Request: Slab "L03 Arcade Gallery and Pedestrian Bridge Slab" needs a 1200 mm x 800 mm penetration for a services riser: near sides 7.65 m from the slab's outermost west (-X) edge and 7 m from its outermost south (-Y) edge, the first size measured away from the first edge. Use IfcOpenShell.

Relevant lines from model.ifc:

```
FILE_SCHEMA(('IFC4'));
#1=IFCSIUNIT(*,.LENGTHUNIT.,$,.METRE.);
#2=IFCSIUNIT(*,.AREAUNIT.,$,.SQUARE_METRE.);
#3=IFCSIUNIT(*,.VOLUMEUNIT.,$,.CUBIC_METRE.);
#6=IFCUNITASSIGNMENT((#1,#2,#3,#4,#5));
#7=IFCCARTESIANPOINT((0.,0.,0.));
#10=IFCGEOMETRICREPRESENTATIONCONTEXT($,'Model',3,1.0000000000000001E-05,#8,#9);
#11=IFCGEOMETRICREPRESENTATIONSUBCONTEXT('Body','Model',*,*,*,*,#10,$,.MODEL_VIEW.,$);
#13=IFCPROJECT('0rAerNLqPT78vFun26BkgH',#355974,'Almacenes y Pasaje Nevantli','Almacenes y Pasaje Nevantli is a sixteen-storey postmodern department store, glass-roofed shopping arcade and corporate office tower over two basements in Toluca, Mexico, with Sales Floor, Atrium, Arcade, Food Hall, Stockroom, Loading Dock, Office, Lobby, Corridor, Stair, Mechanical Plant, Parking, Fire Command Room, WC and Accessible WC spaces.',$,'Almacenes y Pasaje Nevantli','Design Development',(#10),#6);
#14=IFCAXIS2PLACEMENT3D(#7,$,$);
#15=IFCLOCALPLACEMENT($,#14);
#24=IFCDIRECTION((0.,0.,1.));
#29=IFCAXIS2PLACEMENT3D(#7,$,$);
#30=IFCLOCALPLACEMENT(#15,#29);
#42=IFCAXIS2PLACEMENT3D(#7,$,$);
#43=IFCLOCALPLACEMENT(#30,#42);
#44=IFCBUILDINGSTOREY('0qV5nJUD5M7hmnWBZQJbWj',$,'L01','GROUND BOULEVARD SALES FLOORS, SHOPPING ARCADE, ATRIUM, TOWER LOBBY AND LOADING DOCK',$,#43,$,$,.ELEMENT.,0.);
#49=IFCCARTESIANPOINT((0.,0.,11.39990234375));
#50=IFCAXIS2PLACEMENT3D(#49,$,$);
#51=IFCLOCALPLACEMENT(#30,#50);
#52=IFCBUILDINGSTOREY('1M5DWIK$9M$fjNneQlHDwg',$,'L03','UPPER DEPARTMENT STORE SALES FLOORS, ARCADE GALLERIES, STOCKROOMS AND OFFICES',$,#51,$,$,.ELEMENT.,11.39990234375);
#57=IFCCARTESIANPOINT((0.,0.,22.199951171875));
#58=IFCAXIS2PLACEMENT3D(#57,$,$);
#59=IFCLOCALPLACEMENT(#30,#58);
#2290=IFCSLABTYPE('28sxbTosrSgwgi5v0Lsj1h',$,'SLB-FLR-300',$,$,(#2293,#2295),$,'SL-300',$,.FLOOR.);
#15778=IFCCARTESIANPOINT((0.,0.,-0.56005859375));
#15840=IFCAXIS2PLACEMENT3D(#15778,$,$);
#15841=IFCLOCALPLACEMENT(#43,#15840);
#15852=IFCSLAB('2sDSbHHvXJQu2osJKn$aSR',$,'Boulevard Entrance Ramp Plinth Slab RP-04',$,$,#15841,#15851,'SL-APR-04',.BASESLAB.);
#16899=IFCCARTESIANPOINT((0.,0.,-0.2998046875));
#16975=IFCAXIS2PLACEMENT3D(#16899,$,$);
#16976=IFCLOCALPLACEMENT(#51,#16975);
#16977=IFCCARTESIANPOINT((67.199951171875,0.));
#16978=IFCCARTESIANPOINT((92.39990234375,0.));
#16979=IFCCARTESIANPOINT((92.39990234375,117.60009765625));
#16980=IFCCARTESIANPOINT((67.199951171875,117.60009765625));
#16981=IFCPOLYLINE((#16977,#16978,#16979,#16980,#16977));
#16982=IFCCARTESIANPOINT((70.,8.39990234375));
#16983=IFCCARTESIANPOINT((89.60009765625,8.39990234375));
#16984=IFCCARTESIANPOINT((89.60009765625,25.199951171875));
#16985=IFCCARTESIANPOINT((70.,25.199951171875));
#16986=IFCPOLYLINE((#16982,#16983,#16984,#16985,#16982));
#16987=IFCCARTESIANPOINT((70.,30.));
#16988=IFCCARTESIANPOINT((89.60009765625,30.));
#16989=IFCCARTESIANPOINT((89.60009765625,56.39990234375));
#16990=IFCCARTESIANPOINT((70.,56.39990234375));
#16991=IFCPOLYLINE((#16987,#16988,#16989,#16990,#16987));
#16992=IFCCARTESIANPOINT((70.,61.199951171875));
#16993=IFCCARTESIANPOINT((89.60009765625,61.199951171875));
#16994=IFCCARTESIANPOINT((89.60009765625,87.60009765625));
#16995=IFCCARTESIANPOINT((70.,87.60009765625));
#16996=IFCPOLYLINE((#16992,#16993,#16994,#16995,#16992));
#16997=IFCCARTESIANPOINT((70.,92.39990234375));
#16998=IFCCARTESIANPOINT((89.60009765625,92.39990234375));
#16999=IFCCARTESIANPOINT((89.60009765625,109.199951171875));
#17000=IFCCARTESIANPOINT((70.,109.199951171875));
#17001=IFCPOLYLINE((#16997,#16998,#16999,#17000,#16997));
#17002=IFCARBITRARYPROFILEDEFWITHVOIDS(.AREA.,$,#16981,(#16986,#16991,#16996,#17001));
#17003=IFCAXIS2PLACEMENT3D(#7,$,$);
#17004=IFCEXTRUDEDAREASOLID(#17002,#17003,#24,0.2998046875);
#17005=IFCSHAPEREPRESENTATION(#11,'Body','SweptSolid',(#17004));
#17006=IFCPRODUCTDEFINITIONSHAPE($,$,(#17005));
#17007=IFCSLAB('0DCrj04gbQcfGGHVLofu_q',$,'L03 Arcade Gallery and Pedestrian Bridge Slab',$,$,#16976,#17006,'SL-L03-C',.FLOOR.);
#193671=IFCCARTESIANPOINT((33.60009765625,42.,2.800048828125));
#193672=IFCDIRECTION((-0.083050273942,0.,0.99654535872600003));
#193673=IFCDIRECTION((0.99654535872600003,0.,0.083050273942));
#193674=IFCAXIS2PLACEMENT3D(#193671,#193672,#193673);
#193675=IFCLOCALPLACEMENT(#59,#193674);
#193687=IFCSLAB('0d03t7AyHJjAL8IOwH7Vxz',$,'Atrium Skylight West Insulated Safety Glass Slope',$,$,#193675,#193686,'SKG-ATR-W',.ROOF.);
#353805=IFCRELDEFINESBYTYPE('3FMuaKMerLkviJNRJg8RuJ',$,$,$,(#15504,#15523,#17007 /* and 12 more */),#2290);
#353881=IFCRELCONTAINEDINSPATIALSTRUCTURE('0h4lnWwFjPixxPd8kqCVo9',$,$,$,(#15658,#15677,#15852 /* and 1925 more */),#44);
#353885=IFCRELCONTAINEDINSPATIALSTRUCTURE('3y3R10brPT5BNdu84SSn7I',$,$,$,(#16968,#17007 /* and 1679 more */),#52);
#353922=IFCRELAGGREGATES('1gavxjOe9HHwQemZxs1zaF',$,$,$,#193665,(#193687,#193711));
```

```python
import numpy as np
import ifcopenshell
import ifcopenshell.api.feature
import ifcopenshell.api.geometry
import ifcopenshell.api.root
import ifcopenshell.geom
import ifcopenshell.util.placement
import ifcopenshell.util.representation
import ifcopenshell.util.shape
import ifcopenshell.util.unit

model = ifcopenshell.open("model.ifc")
unit_scale = ifcopenshell.util.unit.calculate_unit_scale(model)
settings = ifcopenshell.geom.settings()


def volume(element):
    """Net volume in cubic metres, openings subtracted."""
    shape = ifcopenshell.geom.create_shape(settings, element)
    return ifcopenshell.util.shape.get_volume(shape.geometry)


slab = model.by_guid("0DCrj04gbQcfGGHVLofu_q")
before = volume(slab)

# Extent in the slab's own axes, in metres. The edges named are its -X and -Y sides.
slab_shape = ifcopenshell.geom.create_shape(settings, slab)
vertices = ifcopenshell.util.shape.get_vertices(slab_shape.geometry)
x_min, y_min, bottom = vertices.min(axis=0)
top = vertices[:, 2].max()

opening = ifcopenshell.api.root.create_entity(model, ifc_class="IfcOpeningElement", name="Services riser opening", predefined_type="OPENING")
context = ifcopenshell.util.representation.get_context(model, "Model", "Body", "MODEL_VIEW")
width, depth = 1.2, 0.8
outline = [(0.0, 0.0), (width, 0.0), (width, depth), (0.0, depth), (0.0, 0.0)]
# Overshoot both faces by 50 mm so the cut is clean.
shape = ifcopenshell.api.geometry.add_slab_representation(
    model, context=context, depth=top - bottom + 0.1, polyline=outline
)
ifcopenshell.api.geometry.assign_representation(model, product=opening, representation=shape)

matrix = ifcopenshell.util.placement.get_local_placement(slab.ObjectPlacement)
matrix[:, 3] = matrix @ np.append(np.array([x_min + 7.65, y_min + 7, bottom - 0.05]) / unit_scale, 1.0)
ifcopenshell.api.geometry.edit_object_placement(model, product=opening, matrix=matrix, is_si=False)
ifcopenshell.api.feature.add_feature(model, feature=opening, element=slab)

after = volume(slab)

print(f"slab volume {before:.3f} -> {after:.3f} m3")

model.write("model_edited.ifc")
```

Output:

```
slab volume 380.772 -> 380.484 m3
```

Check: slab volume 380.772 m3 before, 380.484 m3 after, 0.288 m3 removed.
